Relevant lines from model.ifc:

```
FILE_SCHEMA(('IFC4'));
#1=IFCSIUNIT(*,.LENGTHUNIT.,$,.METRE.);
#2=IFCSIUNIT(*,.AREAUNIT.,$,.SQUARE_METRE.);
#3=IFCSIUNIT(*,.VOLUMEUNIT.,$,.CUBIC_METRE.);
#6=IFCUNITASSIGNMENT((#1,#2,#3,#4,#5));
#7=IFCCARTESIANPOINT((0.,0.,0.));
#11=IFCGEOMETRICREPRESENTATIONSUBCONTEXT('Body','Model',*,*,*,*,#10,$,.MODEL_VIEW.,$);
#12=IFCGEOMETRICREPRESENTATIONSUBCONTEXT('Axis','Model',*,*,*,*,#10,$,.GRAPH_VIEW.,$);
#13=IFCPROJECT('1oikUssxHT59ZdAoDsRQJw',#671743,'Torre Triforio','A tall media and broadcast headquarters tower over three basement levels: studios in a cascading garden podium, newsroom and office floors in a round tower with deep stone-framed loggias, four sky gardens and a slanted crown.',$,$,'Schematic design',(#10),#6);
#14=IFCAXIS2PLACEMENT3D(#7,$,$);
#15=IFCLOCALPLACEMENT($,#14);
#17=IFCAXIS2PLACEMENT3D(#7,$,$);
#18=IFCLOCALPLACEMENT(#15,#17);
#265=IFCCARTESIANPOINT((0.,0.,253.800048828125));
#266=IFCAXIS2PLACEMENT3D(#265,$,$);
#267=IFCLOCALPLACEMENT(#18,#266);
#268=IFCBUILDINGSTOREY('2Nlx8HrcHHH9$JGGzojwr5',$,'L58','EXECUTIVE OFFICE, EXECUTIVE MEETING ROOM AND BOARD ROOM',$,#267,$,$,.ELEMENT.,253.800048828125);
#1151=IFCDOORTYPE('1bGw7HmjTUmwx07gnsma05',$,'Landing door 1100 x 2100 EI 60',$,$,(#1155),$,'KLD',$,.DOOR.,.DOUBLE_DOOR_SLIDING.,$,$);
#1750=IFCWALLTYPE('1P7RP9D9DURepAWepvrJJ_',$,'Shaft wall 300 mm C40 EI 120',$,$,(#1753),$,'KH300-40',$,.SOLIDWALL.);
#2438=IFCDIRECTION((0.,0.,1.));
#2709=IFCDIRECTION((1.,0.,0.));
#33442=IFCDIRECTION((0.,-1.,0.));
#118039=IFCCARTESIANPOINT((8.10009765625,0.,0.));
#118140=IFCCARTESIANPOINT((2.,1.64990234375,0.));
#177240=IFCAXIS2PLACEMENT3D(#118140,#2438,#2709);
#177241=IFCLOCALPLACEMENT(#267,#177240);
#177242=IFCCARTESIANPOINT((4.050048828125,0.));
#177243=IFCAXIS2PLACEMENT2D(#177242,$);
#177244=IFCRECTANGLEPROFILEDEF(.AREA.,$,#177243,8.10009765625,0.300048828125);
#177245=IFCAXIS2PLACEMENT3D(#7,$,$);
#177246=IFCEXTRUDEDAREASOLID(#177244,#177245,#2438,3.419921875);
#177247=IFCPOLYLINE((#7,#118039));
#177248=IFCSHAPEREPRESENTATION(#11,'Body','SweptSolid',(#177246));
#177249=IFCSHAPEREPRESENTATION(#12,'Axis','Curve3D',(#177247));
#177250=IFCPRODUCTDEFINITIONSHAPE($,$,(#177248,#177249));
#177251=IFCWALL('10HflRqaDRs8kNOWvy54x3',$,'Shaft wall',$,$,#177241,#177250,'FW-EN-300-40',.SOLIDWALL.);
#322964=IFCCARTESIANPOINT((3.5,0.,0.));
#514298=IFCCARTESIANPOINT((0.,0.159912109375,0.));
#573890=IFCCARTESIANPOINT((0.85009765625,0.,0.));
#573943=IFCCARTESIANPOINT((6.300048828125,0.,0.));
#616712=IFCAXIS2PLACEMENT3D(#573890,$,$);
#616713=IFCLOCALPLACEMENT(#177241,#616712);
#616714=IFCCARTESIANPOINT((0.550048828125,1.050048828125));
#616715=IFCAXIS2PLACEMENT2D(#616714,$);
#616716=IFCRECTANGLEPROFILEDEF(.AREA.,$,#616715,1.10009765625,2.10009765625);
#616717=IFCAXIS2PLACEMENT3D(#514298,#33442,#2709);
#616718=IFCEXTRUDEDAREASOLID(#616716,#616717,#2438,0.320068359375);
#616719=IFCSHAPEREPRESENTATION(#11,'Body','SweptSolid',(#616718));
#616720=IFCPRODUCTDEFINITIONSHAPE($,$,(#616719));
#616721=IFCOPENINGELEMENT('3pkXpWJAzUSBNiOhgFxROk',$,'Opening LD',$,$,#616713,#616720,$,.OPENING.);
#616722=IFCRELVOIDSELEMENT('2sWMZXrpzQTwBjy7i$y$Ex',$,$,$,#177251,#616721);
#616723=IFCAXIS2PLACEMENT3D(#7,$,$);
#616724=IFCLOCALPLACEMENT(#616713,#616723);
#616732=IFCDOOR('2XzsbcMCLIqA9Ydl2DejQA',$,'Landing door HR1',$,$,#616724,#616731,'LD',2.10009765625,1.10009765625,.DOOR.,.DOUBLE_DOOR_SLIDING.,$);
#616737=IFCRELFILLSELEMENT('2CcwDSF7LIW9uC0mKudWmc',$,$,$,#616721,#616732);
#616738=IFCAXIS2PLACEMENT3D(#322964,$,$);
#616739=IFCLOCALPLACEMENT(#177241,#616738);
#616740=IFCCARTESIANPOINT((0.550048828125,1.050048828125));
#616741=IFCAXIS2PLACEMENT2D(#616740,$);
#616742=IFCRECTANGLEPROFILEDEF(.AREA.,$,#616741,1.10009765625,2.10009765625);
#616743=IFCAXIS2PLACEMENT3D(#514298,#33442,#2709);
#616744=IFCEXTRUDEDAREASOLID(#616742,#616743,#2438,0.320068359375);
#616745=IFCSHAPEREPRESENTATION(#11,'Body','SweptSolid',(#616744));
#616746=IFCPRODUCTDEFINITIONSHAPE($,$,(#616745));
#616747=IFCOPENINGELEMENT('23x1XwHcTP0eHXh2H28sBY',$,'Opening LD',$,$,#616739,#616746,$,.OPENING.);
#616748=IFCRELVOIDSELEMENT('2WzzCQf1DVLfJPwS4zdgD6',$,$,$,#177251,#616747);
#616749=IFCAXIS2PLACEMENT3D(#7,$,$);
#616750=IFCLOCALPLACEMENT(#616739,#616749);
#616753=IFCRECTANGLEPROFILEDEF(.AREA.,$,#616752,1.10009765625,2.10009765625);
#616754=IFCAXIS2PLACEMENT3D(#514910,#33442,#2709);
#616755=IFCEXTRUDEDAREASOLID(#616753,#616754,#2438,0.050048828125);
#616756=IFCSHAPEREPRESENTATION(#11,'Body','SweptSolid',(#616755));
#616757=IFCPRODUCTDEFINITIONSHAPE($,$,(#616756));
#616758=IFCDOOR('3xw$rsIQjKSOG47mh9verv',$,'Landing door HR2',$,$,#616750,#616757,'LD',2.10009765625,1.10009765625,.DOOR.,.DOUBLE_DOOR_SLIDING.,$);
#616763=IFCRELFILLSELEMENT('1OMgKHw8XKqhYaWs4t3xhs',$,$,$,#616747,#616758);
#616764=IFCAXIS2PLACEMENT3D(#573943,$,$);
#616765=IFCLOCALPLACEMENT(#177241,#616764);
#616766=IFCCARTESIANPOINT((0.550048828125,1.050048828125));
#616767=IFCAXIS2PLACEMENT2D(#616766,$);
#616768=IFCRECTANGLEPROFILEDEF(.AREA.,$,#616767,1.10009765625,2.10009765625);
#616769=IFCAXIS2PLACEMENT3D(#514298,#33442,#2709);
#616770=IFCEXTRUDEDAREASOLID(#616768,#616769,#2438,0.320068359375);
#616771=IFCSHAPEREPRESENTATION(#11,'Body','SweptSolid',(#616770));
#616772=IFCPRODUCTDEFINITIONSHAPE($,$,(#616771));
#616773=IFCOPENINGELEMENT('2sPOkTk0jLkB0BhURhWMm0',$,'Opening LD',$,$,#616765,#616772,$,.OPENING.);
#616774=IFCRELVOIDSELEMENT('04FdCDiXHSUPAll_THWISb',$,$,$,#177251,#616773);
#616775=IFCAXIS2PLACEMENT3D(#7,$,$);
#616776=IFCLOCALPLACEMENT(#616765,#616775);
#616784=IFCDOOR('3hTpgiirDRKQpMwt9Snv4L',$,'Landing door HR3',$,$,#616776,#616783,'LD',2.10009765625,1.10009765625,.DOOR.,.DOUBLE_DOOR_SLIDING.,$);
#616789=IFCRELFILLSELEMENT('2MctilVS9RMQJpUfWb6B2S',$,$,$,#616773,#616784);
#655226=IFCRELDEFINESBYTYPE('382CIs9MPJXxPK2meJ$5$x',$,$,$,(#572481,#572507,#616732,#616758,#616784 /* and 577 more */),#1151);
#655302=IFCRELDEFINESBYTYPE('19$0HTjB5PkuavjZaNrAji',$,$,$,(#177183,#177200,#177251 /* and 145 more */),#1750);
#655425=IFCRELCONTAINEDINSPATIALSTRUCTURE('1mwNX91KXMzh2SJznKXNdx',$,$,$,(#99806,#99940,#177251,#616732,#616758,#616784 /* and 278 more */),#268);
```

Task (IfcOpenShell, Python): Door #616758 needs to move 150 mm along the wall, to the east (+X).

```python
import ifcopenshell
import ifcopenshell.api.geometry
import ifcopenshell.util.placement
import ifcopenshell.util.unit

model = ifcopenshell.open("model.ifc")
unit_scale = ifcopenshell.util.unit.calculate_unit_scale(model)

door = model.by_guid("3xw$rsIQjKSOG47mh9verv")
opening = door.FillsVoids[0].RelatingOpeningElement
wall = opening.VoidsElements[0].RelatingBuildingElement

wall_matrix = ifcopenshell.util.placement.get_local_placement(wall.ObjectPlacement)
shift = wall_matrix[:3, 0] * 0.15 / unit_scale
before = ifcopenshell.util.placement.get_local_placement(door.ObjectPlacement)[:3, 3].copy()

# The door is placed relative to its opening, so it follows when the opening moves.
matrix = ifcopenshell.util.placement.get_local_placement(opening.ObjectPlacement)
matrix[:3, 3] += shift
ifcopenshell.api.geometry.edit_object_placement(
    model, product=opening, matrix=matrix, is_si=False, should_transform_children=True
)

after = ifcopenshell.util.placement.get_local_placement(door.ObjectPlacement)[:3, 3]
print("door moved by", (after - before).round(3) + 0.0)

model.write("model_v2.ifc")
```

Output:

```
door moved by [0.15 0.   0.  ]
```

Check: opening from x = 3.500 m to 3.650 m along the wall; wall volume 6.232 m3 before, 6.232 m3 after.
